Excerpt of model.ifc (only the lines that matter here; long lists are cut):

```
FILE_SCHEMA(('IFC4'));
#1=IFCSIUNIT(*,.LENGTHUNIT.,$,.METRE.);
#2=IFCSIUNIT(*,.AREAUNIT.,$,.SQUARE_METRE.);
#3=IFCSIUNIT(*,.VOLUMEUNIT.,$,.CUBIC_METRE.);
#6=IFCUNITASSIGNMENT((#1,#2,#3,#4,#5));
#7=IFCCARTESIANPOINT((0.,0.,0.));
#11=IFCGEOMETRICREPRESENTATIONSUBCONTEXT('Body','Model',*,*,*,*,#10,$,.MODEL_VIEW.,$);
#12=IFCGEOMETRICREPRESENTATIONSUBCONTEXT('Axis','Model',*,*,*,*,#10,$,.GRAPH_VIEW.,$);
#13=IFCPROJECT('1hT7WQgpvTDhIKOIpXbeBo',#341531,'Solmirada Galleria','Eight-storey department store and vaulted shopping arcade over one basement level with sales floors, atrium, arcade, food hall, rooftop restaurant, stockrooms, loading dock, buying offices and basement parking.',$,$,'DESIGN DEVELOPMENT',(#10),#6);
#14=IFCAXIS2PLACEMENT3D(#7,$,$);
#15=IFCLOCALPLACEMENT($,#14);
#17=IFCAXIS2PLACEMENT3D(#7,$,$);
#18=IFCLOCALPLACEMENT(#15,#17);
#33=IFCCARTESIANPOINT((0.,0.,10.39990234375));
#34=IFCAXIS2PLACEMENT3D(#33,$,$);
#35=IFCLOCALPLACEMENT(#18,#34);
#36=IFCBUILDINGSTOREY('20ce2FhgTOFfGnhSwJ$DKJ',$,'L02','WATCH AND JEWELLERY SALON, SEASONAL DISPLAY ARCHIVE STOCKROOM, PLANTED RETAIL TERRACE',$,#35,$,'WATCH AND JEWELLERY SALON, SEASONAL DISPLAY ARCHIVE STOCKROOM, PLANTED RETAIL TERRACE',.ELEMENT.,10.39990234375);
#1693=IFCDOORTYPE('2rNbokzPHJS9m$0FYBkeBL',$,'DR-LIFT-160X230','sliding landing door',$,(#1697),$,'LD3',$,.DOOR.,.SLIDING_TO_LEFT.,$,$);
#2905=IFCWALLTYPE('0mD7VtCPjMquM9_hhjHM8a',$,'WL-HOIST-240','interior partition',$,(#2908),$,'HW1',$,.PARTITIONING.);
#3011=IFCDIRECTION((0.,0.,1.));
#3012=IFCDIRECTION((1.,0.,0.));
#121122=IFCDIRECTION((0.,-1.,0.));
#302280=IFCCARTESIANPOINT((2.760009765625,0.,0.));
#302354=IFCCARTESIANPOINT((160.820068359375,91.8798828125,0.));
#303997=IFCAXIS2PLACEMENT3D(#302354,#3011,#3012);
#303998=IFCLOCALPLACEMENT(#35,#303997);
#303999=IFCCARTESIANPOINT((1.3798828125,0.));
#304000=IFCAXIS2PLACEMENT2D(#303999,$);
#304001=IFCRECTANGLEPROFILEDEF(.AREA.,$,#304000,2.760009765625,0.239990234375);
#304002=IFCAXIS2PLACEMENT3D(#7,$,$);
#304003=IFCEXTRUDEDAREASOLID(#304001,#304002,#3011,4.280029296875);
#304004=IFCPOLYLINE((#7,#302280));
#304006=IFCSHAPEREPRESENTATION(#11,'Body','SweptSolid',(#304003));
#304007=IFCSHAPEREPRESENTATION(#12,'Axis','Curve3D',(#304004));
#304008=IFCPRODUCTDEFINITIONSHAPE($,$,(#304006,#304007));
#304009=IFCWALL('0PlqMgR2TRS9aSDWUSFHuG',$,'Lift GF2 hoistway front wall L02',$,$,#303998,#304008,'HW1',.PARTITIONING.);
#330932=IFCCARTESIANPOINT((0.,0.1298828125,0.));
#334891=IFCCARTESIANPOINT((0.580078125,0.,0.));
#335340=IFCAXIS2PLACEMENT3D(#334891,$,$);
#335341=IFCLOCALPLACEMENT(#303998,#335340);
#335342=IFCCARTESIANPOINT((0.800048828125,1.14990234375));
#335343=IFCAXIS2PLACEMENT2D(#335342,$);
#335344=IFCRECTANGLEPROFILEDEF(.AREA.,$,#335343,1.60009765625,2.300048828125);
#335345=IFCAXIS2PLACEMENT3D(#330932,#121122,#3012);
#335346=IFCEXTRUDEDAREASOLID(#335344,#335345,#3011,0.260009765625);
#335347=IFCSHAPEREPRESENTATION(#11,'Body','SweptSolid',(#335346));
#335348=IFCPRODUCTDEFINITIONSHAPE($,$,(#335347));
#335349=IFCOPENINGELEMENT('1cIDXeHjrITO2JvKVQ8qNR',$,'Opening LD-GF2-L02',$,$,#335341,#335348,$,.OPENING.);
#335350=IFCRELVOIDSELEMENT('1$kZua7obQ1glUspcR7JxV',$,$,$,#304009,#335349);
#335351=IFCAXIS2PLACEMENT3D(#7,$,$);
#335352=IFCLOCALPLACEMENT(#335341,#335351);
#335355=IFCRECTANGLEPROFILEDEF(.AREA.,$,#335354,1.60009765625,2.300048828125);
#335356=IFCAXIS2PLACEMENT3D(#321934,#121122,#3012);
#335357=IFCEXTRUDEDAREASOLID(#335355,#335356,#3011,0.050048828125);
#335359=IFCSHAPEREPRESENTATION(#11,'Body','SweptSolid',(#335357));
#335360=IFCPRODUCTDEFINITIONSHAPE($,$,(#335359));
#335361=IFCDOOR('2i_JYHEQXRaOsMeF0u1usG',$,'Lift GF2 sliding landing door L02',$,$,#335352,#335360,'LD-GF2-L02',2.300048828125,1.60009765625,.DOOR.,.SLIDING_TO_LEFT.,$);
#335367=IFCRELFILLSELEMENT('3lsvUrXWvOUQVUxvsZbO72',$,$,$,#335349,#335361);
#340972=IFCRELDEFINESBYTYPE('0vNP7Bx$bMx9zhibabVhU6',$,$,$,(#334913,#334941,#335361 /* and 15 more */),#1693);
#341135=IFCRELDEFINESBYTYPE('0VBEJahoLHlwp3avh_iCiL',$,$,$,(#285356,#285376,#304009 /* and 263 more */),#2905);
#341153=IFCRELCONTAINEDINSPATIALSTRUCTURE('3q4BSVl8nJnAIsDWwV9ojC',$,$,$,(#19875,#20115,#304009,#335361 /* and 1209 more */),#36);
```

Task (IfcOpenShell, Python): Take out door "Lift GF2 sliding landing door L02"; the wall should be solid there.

```python
import ifcopenshell
import ifcopenshell.api.feature
import ifcopenshell.api.root
import ifcopenshell.geom
import ifcopenshell.util.shape

model = ifcopenshell.open("model.ifc")
settings = ifcopenshell.geom.settings()


def volume(element):
    """Net volume in cubic metres, openings subtracted."""
    shape = ifcopenshell.geom.create_shape(settings, element)
    return ifcopenshell.util.shape.get_volume(shape.geometry)


door = model.by_id(335361)
opening = door.FillsVoids[0].RelatingOpeningElement
wall = opening.VoidsElements[0].RelatingBuildingElement
before = volume(wall)

ifcopenshell.api.root.remove_product(model, product=door)
ifcopenshell.api.feature.remove_feature(model, feature=opening)

after = volume(wall)

print(f"wall volume {before:.3f} -> {after:.3f} m3")

model.write("model_updated.ifc")
```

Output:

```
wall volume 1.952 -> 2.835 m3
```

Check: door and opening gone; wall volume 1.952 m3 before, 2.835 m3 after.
